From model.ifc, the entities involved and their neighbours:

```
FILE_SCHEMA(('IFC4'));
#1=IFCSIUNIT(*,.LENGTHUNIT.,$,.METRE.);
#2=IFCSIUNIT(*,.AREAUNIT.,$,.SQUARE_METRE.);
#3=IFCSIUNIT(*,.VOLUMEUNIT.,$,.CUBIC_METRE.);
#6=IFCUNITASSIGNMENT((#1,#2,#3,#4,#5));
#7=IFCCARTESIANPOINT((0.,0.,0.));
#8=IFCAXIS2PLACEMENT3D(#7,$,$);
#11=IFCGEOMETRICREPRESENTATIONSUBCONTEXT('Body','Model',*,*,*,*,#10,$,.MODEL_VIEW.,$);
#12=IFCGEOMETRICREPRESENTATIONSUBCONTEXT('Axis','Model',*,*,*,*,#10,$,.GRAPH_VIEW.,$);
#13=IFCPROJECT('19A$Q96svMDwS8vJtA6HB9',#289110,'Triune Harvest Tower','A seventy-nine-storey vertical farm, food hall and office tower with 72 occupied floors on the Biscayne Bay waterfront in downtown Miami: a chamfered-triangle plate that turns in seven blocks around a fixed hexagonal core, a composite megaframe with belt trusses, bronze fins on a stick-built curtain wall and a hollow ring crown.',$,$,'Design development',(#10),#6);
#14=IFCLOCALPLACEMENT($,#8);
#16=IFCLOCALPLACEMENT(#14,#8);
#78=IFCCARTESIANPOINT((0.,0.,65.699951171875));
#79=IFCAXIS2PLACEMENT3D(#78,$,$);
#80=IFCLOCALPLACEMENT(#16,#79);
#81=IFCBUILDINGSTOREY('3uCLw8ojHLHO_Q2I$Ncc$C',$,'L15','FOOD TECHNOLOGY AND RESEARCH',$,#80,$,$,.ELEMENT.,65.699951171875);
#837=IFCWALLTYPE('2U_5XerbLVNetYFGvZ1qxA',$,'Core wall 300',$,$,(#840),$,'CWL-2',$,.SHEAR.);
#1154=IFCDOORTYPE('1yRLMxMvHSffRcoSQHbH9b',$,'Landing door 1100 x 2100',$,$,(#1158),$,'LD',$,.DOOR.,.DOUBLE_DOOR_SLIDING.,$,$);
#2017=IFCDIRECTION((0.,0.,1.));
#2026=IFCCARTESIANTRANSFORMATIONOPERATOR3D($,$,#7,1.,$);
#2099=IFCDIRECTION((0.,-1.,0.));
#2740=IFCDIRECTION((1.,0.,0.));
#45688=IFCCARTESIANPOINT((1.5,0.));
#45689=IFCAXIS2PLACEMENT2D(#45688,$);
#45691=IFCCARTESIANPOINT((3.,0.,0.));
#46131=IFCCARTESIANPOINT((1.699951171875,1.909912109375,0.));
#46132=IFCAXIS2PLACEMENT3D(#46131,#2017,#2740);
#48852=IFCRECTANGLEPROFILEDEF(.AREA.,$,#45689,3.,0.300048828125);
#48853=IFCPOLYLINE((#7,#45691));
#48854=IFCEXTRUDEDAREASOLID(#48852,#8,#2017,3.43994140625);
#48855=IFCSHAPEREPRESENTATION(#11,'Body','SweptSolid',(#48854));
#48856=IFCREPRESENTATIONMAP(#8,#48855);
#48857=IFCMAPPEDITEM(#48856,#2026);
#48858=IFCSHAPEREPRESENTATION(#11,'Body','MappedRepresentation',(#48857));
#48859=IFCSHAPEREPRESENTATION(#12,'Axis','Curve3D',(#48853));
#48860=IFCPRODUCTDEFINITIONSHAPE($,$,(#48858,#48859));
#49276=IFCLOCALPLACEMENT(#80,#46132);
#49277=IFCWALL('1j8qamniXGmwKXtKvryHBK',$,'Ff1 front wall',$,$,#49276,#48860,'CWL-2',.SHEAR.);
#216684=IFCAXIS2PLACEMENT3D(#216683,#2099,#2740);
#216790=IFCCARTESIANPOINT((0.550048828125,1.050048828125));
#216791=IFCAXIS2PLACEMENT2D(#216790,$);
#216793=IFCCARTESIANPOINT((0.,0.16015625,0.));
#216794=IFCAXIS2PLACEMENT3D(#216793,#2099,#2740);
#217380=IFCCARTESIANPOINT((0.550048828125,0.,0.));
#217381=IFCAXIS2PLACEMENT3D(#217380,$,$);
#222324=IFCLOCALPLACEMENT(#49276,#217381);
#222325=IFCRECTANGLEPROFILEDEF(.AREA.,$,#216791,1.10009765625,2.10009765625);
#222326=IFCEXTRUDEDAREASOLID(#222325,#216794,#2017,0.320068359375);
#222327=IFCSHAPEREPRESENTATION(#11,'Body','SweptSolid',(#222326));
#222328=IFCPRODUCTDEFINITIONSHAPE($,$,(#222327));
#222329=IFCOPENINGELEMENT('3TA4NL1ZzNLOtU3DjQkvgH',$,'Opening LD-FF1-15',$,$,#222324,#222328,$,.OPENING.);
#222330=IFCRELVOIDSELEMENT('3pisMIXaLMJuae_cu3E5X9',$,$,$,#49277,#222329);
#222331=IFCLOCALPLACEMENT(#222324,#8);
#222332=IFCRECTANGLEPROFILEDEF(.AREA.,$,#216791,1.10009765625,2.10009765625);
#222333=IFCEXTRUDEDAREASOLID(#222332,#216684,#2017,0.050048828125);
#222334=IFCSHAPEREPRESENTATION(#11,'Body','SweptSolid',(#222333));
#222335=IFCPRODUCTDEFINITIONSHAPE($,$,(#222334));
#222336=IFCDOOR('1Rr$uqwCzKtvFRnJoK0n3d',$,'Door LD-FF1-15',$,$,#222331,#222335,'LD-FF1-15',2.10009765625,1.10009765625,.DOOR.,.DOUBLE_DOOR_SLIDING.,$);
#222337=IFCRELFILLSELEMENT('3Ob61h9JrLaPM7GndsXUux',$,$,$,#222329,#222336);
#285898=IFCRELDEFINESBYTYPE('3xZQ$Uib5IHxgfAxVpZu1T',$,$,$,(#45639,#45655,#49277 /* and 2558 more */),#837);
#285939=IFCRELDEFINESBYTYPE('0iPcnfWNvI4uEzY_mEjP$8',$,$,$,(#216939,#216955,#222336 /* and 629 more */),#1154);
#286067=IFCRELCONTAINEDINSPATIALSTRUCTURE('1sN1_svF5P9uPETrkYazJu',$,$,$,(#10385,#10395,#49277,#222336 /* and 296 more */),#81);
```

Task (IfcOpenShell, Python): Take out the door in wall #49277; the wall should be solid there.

```python
import ifcopenshell
import ifcopenshell.api.feature
import ifcopenshell.api.root
import ifcopenshell.geom
import ifcopenshell.util.shape

model = ifcopenshell.open("model.ifc")
settings = ifcopenshell.geom.settings()


def volume(element):
    """Net volume in cubic metres, openings subtracted."""
    shape = ifcopenshell.geom.create_shape(settings, element)
    return ifcopenshell.util.shape.get_volume(shape.geometry)


door = model.by_guid("1Rr$uqwCzKtvFRnJoK0n3d")
opening = door.FillsVoids[0].RelatingOpeningElement
wall = opening.VoidsElements[0].RelatingBuildingElement
before = volume(wall)

ifcopenshell.api.root.remove_product(model, product=door)
ifcopenshell.api.feature.remove_feature(model, feature=opening)

after = volume(wall)

print(f"wall volume {before:.3f} -> {after:.3f} m3")

model.write("model_v2.ifc")
```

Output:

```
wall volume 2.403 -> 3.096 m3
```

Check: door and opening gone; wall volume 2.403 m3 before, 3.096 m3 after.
